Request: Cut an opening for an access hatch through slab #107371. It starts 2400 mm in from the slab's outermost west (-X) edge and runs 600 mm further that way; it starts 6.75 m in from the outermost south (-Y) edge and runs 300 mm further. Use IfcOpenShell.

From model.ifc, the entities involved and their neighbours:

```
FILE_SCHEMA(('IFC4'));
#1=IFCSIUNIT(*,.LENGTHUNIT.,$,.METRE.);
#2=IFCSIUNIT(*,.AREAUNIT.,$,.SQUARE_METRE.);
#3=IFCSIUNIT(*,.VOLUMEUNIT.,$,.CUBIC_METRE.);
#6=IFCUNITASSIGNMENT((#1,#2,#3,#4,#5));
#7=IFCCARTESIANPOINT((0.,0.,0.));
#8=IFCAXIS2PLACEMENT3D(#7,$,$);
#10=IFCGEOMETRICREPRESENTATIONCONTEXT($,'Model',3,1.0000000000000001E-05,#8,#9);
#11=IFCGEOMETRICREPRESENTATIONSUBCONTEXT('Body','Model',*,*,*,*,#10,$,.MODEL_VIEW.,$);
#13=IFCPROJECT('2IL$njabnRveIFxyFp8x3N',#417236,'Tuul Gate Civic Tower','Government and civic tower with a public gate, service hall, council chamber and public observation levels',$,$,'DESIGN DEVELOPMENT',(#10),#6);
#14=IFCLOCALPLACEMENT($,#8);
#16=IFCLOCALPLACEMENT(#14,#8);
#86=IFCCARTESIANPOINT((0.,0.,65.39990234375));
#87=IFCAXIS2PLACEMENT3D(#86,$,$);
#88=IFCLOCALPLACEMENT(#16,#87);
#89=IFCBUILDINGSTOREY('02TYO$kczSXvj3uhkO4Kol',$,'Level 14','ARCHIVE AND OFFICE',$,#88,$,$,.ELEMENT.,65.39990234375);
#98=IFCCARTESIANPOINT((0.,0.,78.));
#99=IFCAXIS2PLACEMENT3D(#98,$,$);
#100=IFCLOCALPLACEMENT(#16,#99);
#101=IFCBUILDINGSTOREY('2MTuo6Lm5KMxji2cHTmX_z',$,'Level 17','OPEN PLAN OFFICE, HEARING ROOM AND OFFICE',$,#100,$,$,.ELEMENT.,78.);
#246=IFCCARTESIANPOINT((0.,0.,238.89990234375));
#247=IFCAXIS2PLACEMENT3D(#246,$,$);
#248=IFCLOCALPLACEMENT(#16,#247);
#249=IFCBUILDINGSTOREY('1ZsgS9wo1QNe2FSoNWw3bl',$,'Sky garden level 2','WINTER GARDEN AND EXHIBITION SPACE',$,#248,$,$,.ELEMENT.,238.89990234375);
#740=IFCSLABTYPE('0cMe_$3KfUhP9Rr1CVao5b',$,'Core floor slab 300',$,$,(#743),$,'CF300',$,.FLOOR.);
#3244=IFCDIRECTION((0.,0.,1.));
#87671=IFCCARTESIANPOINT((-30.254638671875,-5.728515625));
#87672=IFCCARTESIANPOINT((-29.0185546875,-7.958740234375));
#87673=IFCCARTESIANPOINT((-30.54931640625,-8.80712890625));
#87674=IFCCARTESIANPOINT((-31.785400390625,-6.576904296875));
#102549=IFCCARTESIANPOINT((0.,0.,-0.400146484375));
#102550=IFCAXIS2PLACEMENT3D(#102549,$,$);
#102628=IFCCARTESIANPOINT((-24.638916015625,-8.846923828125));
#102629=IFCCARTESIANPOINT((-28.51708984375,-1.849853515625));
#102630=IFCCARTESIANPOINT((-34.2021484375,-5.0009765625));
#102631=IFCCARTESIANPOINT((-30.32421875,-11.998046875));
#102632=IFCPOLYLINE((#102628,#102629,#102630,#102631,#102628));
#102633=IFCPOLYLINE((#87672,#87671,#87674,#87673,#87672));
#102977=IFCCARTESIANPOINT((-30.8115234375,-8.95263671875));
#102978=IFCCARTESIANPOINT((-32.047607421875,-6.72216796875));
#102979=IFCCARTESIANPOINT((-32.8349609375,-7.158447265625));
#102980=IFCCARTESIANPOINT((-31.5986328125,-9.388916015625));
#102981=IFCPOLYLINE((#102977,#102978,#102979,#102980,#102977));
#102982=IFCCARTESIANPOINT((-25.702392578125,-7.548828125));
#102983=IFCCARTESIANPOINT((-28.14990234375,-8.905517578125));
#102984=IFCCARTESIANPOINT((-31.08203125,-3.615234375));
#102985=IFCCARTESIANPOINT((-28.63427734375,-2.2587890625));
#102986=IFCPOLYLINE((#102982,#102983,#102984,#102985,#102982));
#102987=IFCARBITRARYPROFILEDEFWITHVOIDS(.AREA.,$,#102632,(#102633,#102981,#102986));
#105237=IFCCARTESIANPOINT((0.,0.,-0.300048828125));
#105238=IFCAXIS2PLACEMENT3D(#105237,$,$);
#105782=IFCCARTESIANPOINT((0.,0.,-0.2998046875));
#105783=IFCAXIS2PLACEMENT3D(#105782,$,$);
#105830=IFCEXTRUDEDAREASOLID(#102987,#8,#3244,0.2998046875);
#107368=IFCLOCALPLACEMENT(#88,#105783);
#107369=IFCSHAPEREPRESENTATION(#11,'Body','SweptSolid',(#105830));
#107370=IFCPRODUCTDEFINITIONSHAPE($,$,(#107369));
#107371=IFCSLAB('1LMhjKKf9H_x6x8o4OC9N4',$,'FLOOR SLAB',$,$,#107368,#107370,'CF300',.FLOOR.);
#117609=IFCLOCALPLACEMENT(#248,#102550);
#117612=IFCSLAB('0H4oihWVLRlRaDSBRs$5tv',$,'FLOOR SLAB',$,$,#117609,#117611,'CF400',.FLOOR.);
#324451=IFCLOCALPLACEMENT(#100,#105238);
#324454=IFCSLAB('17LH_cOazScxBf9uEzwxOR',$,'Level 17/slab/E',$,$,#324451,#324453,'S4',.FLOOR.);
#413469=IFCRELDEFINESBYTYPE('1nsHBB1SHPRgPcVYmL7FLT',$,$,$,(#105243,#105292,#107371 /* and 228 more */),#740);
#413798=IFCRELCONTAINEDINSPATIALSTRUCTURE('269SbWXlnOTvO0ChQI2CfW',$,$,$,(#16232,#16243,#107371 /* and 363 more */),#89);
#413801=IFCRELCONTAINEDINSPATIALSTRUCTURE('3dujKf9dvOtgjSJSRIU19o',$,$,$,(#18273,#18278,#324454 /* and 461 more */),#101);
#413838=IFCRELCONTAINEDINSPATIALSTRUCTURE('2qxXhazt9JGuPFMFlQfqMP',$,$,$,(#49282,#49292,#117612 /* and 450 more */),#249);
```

```python
import numpy as np
import ifcopenshell
import ifcopenshell.api.feature
import ifcopenshell.api.geometry
import ifcopenshell.api.root
import ifcopenshell.geom
import ifcopenshell.util.placement
import ifcopenshell.util.representation
import ifcopenshell.util.shape
import ifcopenshell.util.unit

model = ifcopenshell.open("model.ifc")
unit_scale = ifcopenshell.util.unit.calculate_unit_scale(model)
settings = ifcopenshell.geom.settings()


def volume(element):
    """Net volume in cubic metres, openings subtracted."""
    shape = ifcopenshell.geom.create_shape(settings, element)
    return ifcopenshell.util.shape.get_volume(shape.geometry)


slab = model.by_guid("1LMhjKKf9H_x6x8o4OC9N4")
before = volume(slab)

# Extent in the slab's own axes, in metres. The edges named are its -X and -Y sides.
slab_shape = ifcopenshell.geom.create_shape(settings, slab)
vertices = ifcopenshell.util.shape.get_vertices(slab_shape.geometry)
x_min, y_min, bottom = vertices.min(axis=0)
top = vertices[:, 2].max()

opening = ifcopenshell.api.root.create_entity(model, ifc_class="IfcOpeningElement", name="Access hatch opening", predefined_type="OPENING")
context = ifcopenshell.util.representation.get_context(model, "Model", "Body", "MODEL_VIEW")
width, depth = 0.6, 0.3
outline = [(0.0, 0.0), (width, 0.0), (width, depth), (0.0, depth), (0.0, 0.0)]
# Overshoot both faces by 50 mm so the cut is clean.
shape = ifcopenshell.api.geometry.add_slab_representation(
    model, context=context, depth=top - bottom + 0.1, polyline=outline
)
ifcopenshell.api.geometry.assign_representation(model, product=opening, representation=shape)

matrix = ifcopenshell.util.placement.get_local_placement(slab.ObjectPlacement)
matrix[:, 3] = matrix @ np.append(np.array([x_min + 2.4, y_min + 6.75, bottom - 0.05]) / unit_scale, 1.0)
ifcopenshell.api.geometry.edit_object_placement(model, product=opening, matrix=matrix, is_si=False)
ifcopenshell.api.feature.add_feature(model, feature=opening, element=slab)

after = volume(slab)

print(f"slab volume {before:.3f} -> {after:.3f} m3")

model.write("model_v2.ifc")
```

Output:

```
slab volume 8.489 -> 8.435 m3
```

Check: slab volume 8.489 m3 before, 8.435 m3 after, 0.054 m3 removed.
